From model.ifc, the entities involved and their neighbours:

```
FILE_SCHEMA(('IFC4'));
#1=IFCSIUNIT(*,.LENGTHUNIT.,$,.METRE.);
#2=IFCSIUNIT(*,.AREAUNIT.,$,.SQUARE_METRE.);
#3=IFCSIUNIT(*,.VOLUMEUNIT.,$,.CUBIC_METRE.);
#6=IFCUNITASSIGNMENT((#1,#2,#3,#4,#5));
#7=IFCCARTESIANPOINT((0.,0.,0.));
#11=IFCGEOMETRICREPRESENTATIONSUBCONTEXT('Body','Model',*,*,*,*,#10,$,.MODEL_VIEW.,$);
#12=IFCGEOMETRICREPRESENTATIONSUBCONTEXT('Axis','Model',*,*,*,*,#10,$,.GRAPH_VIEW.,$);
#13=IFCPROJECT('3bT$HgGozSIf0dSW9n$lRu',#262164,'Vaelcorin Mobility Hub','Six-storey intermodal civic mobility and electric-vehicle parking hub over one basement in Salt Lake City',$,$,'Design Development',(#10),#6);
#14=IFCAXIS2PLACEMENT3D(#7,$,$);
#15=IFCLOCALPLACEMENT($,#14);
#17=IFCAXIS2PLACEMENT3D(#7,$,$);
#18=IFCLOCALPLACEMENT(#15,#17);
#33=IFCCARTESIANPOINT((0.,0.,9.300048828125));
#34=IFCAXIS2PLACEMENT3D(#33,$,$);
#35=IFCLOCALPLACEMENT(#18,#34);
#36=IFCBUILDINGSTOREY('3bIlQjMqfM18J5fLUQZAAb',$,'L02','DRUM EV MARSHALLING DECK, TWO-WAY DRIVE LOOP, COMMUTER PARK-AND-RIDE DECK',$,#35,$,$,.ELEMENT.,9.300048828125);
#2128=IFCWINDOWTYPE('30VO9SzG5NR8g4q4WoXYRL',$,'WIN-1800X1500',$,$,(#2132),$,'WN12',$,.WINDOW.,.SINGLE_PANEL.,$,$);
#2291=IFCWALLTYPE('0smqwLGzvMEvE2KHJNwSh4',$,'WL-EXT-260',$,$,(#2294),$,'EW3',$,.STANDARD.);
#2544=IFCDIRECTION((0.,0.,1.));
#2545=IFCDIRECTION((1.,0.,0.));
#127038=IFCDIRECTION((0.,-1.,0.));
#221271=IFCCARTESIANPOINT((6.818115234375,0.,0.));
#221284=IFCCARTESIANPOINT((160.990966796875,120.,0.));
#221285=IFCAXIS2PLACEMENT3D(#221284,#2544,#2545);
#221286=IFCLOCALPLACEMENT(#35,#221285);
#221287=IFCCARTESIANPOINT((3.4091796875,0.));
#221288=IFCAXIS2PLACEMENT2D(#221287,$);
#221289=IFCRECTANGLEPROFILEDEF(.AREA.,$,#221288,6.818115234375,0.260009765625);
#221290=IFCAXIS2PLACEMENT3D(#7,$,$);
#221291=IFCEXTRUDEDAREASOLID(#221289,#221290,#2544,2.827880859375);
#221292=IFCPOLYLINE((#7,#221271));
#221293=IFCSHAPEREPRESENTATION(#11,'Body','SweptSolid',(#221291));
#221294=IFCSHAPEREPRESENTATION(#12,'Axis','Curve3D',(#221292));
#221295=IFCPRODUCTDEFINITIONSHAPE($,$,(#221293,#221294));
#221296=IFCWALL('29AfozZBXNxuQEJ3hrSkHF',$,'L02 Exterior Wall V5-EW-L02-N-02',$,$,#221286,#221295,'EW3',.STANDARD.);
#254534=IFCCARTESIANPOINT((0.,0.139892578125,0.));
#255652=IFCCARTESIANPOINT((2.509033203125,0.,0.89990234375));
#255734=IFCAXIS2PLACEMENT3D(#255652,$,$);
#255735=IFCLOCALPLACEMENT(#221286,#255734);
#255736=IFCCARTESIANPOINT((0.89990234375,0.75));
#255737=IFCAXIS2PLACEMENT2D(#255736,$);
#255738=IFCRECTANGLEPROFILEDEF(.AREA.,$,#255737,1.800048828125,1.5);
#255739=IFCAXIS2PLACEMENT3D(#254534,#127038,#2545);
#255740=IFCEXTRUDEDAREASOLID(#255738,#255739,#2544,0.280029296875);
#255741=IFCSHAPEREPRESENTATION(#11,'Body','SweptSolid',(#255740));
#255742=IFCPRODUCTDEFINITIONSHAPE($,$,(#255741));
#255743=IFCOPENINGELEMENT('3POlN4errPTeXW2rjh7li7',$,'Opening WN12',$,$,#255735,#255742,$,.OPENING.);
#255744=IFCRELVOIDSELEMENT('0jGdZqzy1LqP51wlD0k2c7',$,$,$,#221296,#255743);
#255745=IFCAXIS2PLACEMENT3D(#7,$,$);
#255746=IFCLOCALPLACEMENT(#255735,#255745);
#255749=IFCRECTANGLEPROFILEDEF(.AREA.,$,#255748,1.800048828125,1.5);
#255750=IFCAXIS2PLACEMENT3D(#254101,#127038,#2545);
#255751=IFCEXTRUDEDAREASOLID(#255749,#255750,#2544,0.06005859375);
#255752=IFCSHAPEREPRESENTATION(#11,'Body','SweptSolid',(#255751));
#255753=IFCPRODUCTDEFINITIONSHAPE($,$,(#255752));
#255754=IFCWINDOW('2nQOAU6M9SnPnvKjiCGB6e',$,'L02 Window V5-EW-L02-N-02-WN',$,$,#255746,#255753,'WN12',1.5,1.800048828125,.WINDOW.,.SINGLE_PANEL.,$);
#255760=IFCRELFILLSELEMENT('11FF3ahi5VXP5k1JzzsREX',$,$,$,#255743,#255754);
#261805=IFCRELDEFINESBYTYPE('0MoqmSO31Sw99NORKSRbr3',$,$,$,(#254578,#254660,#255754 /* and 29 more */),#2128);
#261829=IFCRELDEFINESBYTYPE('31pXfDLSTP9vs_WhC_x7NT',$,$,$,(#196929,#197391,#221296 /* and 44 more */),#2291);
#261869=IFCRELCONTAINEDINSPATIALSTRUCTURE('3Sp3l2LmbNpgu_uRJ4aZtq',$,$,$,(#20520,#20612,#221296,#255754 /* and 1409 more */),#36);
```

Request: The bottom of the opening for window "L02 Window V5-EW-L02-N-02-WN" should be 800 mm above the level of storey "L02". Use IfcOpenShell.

```python
import numpy as np
import ifcopenshell
import ifcopenshell.api.geometry
import ifcopenshell.geom
import ifcopenshell.util.element
import ifcopenshell.util.placement
import ifcopenshell.util.shape
import ifcopenshell.util.unit

model = ifcopenshell.open("model.ifc")
unit_scale = ifcopenshell.util.unit.calculate_unit_scale(model)

window = model.by_id(255754)
opening = window.FillsVoids[0].RelatingOpeningElement
storey = ifcopenshell.util.element.get_container(window, ifc_class="IfcBuildingStorey")
level = ifcopenshell.util.placement.get_local_placement(storey.ObjectPlacement)[2, 3]

# The opening's origin need not be at the sill, so measure its lowest point.
shape = ifcopenshell.geom.create_shape(ifcopenshell.geom.settings(), opening)
bottom = ifcopenshell.util.shape.get_shape_bottom_elevation(shape, shape.geometry) / unit_scale
dz = level + 0.8 / unit_scale - bottom

shift = np.array([0.0, 0.0, dz])
# The window is placed relative to its opening, so it follows when the opening moves.
matrix = ifcopenshell.util.placement.get_local_placement(opening.ObjectPlacement)
matrix[:3, 3] += shift
ifcopenshell.api.geometry.edit_object_placement(
    model, product=opening, matrix=matrix, is_si=False, should_transform_children=True
)

print(f"moved by {dz * unit_scale:+.3f} m")

model.write("model_v2.ifc")
```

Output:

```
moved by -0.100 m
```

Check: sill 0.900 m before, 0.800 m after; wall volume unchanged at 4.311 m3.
